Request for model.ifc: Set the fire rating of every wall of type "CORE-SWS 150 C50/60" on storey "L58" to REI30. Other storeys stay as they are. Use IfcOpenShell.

First a look at what the model holds.

```python
import ifcopenshell
import ifcopenshell.util.element

model = ifcopenshell.open("model.ifc")
print(model.schema)
storey = next(s for s in model.by_type("IfcBuildingStorey") if s.Name == "L58")
walls = [e for e in ifcopenshell.util.element.get_decomposition(storey) if e.is_a("IfcWall")]
seen = {}
for e in walls:
    element_type = ifcopenshell.util.element.get_type(e)
    key = (element_type.Name if element_type != e and element_type else None, ifcopenshell.util.element.get_pset(e, "Pset_WallCommon", "FireRating"))
    seen[key] = seen.get(key, 0) + 1
for (name, value), count in sorted(seen.items(), key=str):
    print(count, "x", name, "|", value)
```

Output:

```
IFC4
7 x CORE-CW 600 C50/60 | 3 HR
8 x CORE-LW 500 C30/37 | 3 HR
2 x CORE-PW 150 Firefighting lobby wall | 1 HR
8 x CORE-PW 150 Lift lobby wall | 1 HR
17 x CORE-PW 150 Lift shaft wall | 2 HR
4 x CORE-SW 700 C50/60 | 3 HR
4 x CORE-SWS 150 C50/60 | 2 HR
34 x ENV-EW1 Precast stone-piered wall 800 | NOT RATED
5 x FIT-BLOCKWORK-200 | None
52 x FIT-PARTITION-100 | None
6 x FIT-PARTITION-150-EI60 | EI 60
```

```python
import ifcopenshell
import ifcopenshell.api.pset
import ifcopenshell.util.element

model = ifcopenshell.open("model.ifc")

storey = next(s for s in model.by_type("IfcBuildingStorey") if s.Name == "L58")
walls = [e for e in ifcopenshell.util.element.get_decomposition(storey) if e.is_a("IfcWall")]

count = 0
for e in walls:
    element_type = ifcopenshell.util.element.get_type(e)
    if element_type in (None, e) or element_type.Name != "CORE-SWS 150 C50/60":
        continue
    found = ifcopenshell.util.element.get_pset(e, "Pset_WallCommon", should_inherit=False)
    if found:
        pset = model.by_id(found["id"])
        if len(ifcopenshell.util.element.get_elements_by_pset(pset)) > 1:
            pset = ifcopenshell.api.pset.unshare_pset(model, products=[e], pset=pset)[0]
    else:
        pset = ifcopenshell.api.pset.add_pset(model, product=e, name="Pset_WallCommon")
    ifcopenshell.api.pset.edit_pset(model, pset=pset, properties={"FireRating": "REI30"})
    count += 1

print(count, "walls updated")

model.write("model-out.ifc")
```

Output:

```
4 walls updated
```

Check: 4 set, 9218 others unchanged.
